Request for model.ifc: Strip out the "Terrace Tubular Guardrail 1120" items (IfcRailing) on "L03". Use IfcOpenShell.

First a look at what the model holds.

```python
import ifcopenshell
import ifcopenshell.util.element

model = ifcopenshell.open("model.ifc")
print(model.schema)
storey = next(s for s in model.by_type("IfcBuildingStorey") if s.Name == "L03")
railings = [e for e in ifcopenshell.util.element.get_decomposition(storey) if e.is_a("IfcRailing")]
seen = {}
for e in railings:
    element_type = ifcopenshell.util.element.get_type(e)
    name = element_type.Name if element_type not in (None, e) else None
    seen[name] = seen.get(name, 0) + 1
for name, count in sorted(seen.items(), key=str):
    print(count, "x", name)
```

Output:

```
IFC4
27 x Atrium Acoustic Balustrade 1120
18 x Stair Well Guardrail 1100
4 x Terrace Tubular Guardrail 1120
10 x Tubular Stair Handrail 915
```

```python
import ifcopenshell
import ifcopenshell.api.root
import ifcopenshell.util.element

model = ifcopenshell.open("model.ifc")

storey = next(s for s in model.by_type("IfcBuildingStorey") if s.Name == "L03")
railings = [e for e in ifcopenshell.util.element.get_decomposition(storey) if e.is_a("IfcRailing")]
targets = [e for e in railings if (t := ifcopenshell.util.element.get_type(e)) not in (None, e) and t.Name == "Terrace Tubular Guardrail 1120"]

for e in targets:
    ifcopenshell.api.root.remove_product(model, product=e)
print(len(targets), "removed")

model.write("model_updated.ifc")
```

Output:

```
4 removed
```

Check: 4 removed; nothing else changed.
